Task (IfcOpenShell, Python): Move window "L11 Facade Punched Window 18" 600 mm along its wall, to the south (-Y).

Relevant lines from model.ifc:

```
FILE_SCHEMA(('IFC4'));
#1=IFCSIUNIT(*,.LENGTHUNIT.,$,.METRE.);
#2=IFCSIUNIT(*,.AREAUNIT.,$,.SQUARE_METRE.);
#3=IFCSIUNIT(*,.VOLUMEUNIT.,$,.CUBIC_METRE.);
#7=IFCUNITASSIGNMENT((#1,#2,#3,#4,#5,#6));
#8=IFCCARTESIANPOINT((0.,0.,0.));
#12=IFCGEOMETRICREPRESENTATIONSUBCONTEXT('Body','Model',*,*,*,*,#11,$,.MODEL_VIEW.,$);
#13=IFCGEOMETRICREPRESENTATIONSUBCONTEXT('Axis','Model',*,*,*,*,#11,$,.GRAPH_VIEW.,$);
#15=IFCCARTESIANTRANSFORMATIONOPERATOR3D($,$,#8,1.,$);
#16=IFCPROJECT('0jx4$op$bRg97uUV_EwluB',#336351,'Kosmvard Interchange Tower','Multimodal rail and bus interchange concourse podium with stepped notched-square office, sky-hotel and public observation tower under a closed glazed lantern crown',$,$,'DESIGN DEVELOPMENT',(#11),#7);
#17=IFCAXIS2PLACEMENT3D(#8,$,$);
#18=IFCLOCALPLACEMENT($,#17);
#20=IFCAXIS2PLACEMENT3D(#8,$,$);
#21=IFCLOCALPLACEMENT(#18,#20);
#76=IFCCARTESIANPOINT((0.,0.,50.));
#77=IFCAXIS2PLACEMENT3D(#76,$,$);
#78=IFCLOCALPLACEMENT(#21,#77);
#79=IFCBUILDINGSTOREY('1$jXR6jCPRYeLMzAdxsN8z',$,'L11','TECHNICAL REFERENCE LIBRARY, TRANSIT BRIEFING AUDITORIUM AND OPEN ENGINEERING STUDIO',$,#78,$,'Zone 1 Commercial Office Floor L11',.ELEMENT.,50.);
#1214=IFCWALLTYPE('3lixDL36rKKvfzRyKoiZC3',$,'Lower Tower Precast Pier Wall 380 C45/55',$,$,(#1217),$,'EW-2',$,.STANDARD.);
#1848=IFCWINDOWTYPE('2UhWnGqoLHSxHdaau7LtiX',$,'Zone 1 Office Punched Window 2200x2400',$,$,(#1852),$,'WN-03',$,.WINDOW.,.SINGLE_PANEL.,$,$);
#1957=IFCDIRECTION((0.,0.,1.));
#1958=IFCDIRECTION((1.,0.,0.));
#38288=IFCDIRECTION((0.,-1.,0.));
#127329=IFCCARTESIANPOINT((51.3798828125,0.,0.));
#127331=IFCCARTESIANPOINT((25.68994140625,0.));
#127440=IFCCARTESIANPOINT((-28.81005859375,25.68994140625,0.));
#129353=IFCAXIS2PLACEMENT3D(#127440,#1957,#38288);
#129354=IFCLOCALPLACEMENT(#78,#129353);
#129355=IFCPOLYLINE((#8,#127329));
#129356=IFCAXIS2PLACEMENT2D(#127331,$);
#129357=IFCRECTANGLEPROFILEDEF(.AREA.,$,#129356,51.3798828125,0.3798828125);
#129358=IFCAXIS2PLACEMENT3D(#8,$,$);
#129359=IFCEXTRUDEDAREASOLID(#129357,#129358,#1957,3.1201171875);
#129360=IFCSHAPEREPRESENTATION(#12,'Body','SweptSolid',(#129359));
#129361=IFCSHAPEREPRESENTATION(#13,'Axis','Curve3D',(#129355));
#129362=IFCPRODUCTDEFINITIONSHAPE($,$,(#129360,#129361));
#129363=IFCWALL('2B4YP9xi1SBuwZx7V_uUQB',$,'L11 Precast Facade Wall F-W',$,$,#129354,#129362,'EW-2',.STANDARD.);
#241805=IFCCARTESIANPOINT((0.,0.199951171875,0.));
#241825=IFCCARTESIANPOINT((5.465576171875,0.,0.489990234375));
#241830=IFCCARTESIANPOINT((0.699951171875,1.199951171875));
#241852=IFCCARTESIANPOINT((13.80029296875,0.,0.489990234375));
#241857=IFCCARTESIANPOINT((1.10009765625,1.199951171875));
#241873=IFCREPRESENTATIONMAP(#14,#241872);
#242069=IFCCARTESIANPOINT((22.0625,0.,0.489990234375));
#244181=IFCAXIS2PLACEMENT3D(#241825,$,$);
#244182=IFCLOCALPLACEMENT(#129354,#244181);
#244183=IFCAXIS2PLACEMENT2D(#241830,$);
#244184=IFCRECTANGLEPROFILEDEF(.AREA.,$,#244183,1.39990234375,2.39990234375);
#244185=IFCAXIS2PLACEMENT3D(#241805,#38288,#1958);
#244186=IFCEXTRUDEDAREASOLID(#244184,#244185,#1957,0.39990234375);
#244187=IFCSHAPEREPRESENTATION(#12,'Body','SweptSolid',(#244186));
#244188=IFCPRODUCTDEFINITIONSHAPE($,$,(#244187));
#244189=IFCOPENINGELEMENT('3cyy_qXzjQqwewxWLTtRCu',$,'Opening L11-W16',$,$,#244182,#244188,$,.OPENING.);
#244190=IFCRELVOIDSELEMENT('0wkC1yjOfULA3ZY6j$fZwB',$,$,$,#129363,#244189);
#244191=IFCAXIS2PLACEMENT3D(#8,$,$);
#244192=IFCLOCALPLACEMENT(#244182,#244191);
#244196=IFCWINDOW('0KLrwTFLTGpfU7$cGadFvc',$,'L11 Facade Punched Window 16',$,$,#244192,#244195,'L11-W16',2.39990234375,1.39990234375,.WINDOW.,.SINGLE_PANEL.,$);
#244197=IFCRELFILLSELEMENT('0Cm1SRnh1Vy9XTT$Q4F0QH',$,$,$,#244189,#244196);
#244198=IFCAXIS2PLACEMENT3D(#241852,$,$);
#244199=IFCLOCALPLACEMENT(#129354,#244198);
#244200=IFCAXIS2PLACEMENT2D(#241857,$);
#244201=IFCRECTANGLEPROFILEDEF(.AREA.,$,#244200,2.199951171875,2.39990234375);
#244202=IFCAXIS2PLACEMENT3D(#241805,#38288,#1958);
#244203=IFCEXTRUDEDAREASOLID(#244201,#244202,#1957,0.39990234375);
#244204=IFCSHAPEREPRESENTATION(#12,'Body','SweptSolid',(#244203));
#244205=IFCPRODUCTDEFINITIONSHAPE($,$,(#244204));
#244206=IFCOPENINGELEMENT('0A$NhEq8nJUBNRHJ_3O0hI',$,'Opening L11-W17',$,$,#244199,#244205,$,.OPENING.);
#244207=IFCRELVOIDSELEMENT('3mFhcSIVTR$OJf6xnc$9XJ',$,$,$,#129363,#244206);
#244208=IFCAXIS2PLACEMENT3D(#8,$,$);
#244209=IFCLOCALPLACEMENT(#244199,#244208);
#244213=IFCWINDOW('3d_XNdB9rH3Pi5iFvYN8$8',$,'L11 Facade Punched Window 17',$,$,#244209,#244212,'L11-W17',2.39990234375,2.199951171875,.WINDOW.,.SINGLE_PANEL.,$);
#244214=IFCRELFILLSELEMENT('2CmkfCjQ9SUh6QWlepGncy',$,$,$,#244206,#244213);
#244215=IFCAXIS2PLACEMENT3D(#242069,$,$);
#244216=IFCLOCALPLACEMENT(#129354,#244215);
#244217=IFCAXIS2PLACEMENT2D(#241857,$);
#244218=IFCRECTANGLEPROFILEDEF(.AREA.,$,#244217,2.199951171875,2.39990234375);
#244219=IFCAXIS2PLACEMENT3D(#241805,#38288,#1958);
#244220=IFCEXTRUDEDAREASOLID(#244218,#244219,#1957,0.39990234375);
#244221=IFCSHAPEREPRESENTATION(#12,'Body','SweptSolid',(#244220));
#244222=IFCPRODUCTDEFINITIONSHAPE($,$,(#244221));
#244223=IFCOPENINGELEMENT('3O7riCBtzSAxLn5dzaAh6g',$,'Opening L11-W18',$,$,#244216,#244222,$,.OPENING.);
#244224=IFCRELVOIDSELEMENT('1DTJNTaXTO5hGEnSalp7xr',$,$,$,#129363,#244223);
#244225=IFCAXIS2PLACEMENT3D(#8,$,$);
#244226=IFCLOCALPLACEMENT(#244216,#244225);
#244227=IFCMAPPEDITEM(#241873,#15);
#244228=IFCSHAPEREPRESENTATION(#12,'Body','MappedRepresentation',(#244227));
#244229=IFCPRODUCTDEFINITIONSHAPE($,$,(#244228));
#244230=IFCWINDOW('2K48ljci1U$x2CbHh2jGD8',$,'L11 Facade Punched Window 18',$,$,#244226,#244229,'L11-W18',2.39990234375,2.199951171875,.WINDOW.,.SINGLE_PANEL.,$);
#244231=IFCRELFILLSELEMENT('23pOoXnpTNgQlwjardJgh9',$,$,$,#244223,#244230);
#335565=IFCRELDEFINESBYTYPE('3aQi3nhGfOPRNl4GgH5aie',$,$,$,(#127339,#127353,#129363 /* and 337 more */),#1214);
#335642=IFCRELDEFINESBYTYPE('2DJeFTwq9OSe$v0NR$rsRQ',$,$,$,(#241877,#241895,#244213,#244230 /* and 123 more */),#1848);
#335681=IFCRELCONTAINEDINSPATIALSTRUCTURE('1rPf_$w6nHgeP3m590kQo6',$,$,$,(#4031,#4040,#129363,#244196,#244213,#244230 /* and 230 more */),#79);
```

```python
import ifcopenshell
import ifcopenshell.api.geometry
import ifcopenshell.util.placement
import ifcopenshell.util.unit

model = ifcopenshell.open("model.ifc")
unit_scale = ifcopenshell.util.unit.calculate_unit_scale(model)

window = model.by_guid("2K48ljci1U$x2CbHh2jGD8")
opening = window.FillsVoids[0].RelatingOpeningElement
wall = opening.VoidsElements[0].RelatingBuildingElement

wall_matrix = ifcopenshell.util.placement.get_local_placement(wall.ObjectPlacement)
shift = wall_matrix[:3, 0] * 0.6 / unit_scale
before = ifcopenshell.util.placement.get_local_placement(window.ObjectPlacement)[:3, 3].copy()

# The window is placed relative to its opening, so it follows when the opening moves.
matrix = ifcopenshell.util.placement.get_local_placement(opening.ObjectPlacement)
matrix[:3, 3] += shift
ifcopenshell.api.geometry.edit_object_placement(
    model, product=opening, matrix=matrix, is_si=False, should_transform_children=True
)

after = ifcopenshell.util.placement.get_local_placement(window.ObjectPlacement)[:3, 3]
print("window moved by", (after - before).round(3) + 0.0)

model.write("model-out.ifc")
```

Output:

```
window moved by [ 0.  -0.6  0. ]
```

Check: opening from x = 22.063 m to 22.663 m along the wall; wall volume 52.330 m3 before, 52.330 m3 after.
